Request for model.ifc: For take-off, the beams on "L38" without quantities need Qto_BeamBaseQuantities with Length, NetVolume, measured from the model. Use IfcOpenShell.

First a look at what the model holds.

```python
import ifcopenshell
import ifcopenshell.util.element
import ifcopenshell.util.unit

model = ifcopenshell.open("model.ifc")
print(model.schema)
for unit_type in ("LENGTHUNIT", "AREAUNIT", "VOLUMEUNIT"):
    print(unit_type, ifcopenshell.util.unit.calculate_unit_scale(model, unit_type))
storey = next(s for s in model.by_type("IfcBuildingStorey") if s.Name == "L38")
beams = [e for e in ifcopenshell.util.element.get_decomposition(storey) if e.is_a("IfcBeam")]
for e in sorted(beams, key=lambda e: e.id()):
    print(e.id(), e.is_a(), e.Name, list(ifcopenshell.util.element.get_psets(e, qtos_only=True)), sep=" | ")
```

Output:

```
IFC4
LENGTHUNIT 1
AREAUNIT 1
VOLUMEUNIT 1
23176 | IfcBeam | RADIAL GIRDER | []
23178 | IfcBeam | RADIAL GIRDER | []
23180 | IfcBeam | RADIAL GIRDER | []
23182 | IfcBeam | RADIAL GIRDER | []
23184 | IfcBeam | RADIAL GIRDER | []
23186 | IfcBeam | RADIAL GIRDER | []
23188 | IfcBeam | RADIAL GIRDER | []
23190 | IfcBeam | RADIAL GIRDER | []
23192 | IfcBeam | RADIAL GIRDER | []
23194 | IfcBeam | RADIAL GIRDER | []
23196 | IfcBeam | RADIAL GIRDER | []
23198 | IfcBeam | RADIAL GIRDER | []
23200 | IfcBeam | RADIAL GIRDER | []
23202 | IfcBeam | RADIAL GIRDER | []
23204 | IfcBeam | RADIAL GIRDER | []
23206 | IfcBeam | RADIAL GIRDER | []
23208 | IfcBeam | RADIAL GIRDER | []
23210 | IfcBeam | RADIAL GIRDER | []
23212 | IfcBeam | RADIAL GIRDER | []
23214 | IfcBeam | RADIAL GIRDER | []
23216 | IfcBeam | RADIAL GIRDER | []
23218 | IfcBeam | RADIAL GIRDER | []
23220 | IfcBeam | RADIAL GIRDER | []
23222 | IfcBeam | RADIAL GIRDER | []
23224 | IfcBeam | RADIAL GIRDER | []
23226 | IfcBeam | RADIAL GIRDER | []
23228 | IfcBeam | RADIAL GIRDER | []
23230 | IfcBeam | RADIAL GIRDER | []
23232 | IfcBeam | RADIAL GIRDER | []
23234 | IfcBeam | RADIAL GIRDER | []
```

```python
import ifcopenshell
import ifcopenshell.api.pset
import ifcopenshell.geom
import ifcopenshell.util.element
import ifcopenshell.util.shape
import ifcopenshell.util.unit

model = ifcopenshell.open("model.ifc")
unit_scale = ifcopenshell.util.unit.calculate_unit_scale(model)
volume_scale = ifcopenshell.util.unit.calculate_unit_scale(model, "VOLUMEUNIT")
settings = ifcopenshell.geom.settings()

storey = next(s for s in model.by_type("IfcBuildingStorey") if s.Name == "L38")
beams = [e for e in ifcopenshell.util.element.get_decomposition(storey) if e.is_a("IfcBeam")]

for e in sorted(beams, key=lambda e: e.id()):
    if ifcopenshell.util.element.get_psets(e, qtos_only=True, should_inherit=False):
        continue
    # Geometry comes back in metres, in the element's own axes.
    shape = ifcopenshell.geom.create_shape(settings, e)
    values = {
        "Length": ifcopenshell.util.shape.get_max_xyz(shape.geometry) / unit_scale,
        "NetVolume": ifcopenshell.util.shape.get_volume(shape.geometry) / volume_scale,
    }
    qto = ifcopenshell.api.pset.add_qto(model, product=e, name="Qto_BeamBaseQuantities")
    ifcopenshell.api.pset.edit_qto(model, qto=qto, properties=values)
    print(e.id(), {k: round(v, 3) for k, v in values.items()})

model.write("model_updated.ifc")
```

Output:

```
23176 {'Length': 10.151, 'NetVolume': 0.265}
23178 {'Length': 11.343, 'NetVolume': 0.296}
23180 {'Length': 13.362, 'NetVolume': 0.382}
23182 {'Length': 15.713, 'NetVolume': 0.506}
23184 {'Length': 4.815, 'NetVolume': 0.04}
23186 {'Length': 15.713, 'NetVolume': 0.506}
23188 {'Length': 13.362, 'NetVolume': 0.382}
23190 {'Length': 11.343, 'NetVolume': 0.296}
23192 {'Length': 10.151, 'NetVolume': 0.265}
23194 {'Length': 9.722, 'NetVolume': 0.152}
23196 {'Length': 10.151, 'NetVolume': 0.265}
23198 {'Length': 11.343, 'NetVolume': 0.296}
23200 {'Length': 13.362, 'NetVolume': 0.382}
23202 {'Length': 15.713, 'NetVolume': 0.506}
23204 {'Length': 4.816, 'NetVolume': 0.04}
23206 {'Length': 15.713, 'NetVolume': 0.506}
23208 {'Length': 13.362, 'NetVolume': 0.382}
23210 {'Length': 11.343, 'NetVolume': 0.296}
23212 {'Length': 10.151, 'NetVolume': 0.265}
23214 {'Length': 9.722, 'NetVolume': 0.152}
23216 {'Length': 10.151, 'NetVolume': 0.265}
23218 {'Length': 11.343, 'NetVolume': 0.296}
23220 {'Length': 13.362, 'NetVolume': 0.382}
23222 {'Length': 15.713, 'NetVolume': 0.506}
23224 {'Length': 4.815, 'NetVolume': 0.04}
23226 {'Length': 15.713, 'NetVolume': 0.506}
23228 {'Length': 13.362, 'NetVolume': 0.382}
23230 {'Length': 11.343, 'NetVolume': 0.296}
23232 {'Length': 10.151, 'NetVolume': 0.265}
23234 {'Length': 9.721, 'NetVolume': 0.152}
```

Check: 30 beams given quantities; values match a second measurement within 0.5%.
